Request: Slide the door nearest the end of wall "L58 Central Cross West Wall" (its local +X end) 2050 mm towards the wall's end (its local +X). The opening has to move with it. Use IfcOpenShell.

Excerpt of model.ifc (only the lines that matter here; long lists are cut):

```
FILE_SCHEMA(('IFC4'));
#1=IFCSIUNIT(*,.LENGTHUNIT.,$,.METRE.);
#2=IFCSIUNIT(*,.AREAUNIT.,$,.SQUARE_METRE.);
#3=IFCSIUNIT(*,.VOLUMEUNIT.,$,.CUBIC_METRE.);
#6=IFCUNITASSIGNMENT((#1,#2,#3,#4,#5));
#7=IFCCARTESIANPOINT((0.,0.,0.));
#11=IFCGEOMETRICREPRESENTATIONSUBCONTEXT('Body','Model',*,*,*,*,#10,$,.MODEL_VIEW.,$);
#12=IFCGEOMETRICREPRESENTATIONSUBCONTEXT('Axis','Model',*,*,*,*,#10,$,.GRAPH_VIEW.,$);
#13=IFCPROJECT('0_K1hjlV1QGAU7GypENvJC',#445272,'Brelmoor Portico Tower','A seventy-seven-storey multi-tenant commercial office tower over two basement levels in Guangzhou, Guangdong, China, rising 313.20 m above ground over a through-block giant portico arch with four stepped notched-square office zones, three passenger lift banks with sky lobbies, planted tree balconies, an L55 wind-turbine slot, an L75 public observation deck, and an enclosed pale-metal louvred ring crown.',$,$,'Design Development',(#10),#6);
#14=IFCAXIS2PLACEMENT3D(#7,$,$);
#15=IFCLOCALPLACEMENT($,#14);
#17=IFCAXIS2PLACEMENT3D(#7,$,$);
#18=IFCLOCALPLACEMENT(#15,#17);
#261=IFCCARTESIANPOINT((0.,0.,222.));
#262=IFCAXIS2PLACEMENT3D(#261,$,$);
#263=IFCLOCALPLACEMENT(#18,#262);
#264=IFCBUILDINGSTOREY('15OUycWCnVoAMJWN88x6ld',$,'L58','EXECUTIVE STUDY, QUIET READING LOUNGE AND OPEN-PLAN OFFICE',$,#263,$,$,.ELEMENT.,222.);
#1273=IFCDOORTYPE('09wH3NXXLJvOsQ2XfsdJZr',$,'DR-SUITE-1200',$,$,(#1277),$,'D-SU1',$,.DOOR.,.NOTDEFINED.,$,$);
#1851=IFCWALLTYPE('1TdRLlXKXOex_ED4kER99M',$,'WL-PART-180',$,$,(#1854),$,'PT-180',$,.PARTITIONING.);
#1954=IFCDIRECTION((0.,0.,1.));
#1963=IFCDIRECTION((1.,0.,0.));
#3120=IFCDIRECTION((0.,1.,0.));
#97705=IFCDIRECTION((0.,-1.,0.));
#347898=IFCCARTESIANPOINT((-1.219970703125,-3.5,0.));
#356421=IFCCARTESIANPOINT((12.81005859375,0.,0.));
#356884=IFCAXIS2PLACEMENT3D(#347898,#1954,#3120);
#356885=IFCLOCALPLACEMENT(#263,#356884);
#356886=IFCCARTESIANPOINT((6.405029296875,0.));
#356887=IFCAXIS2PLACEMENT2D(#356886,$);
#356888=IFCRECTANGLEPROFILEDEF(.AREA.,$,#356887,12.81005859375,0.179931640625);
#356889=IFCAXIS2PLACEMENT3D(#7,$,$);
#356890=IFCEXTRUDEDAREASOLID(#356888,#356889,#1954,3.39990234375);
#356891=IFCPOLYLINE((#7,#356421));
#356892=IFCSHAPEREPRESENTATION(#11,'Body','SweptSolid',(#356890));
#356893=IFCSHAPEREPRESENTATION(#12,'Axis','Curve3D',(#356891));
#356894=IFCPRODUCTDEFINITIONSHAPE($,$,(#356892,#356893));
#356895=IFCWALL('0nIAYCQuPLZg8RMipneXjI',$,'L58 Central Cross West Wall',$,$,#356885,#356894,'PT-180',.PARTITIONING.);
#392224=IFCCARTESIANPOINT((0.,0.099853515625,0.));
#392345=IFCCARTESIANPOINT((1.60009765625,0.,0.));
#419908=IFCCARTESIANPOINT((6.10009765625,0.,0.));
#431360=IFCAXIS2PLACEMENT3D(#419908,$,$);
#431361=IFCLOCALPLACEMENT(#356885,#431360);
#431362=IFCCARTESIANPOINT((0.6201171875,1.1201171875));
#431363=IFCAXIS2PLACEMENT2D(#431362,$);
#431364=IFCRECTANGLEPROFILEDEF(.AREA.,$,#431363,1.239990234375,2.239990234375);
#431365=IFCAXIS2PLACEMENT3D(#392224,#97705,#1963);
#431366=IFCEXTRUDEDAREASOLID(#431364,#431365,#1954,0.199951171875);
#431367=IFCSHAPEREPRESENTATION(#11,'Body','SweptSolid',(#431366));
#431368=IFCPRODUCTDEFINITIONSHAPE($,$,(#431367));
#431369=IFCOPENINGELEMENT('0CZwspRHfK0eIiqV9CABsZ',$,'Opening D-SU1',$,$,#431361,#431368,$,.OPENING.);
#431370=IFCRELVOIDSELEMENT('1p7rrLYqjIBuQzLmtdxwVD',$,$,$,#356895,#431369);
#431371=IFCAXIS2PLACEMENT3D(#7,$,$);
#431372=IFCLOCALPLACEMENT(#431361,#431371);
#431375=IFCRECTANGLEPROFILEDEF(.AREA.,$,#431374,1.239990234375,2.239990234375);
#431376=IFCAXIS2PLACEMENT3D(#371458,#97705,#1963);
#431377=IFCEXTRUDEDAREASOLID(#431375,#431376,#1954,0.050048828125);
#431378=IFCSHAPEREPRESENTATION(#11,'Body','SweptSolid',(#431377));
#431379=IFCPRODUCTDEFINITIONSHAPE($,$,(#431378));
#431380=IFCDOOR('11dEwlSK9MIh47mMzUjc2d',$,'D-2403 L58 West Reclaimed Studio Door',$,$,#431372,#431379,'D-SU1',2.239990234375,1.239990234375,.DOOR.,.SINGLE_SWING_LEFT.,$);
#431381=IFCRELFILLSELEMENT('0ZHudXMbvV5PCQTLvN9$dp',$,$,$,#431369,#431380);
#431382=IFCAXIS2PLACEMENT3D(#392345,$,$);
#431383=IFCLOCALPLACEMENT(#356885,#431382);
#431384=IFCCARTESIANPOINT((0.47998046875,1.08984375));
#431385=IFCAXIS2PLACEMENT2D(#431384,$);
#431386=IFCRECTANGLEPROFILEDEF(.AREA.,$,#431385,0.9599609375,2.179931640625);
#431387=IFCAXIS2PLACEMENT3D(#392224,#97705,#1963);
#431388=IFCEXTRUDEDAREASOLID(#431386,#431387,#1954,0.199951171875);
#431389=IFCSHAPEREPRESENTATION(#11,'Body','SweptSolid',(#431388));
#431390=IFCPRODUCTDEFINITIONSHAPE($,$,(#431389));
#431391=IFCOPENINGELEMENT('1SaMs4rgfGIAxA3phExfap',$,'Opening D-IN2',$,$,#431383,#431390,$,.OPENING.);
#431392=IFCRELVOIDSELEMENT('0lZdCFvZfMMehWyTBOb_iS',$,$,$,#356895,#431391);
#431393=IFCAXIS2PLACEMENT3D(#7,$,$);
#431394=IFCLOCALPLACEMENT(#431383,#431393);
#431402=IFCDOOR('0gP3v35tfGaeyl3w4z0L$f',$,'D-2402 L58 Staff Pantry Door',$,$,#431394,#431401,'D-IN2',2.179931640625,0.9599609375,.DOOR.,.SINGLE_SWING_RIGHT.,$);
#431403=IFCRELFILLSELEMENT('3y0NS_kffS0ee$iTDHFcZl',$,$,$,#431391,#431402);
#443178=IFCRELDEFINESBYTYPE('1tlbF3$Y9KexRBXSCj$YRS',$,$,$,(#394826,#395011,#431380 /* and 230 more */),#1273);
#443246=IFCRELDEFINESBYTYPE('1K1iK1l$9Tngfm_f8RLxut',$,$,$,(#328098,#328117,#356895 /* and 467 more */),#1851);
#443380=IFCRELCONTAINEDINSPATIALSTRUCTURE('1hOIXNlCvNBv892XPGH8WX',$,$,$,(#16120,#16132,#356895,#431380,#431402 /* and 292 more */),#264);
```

```python
import ifcopenshell
import ifcopenshell.api.geometry
import ifcopenshell.util.placement

model = ifcopenshell.open("model.ifc")

door = model.by_guid("11dEwlSK9MIh47mMzUjc2d")
opening = door.FillsVoids[0].RelatingOpeningElement
wall = opening.VoidsElements[0].RelatingBuildingElement

wall_matrix = ifcopenshell.util.placement.get_local_placement(wall.ObjectPlacement)
shift = wall_matrix[:3, 0] * 2.05
before = ifcopenshell.util.placement.get_local_placement(door.ObjectPlacement)[:3, 3].copy()

# The door is placed relative to its opening, so it follows when the opening moves.
matrix = ifcopenshell.util.placement.get_local_placement(opening.ObjectPlacement)
matrix[:3, 3] += shift
ifcopenshell.api.geometry.edit_object_placement(
    model, product=opening, matrix=matrix, is_si=False, should_transform_children=True
)

after = ifcopenshell.util.placement.get_local_placement(door.ObjectPlacement)[:3, 3]
print("door moved by", (after - before).round(3) + 0.0)

model.write("model_rev.ifc")
```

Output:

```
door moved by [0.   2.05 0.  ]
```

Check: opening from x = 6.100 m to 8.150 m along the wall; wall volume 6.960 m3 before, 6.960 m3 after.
